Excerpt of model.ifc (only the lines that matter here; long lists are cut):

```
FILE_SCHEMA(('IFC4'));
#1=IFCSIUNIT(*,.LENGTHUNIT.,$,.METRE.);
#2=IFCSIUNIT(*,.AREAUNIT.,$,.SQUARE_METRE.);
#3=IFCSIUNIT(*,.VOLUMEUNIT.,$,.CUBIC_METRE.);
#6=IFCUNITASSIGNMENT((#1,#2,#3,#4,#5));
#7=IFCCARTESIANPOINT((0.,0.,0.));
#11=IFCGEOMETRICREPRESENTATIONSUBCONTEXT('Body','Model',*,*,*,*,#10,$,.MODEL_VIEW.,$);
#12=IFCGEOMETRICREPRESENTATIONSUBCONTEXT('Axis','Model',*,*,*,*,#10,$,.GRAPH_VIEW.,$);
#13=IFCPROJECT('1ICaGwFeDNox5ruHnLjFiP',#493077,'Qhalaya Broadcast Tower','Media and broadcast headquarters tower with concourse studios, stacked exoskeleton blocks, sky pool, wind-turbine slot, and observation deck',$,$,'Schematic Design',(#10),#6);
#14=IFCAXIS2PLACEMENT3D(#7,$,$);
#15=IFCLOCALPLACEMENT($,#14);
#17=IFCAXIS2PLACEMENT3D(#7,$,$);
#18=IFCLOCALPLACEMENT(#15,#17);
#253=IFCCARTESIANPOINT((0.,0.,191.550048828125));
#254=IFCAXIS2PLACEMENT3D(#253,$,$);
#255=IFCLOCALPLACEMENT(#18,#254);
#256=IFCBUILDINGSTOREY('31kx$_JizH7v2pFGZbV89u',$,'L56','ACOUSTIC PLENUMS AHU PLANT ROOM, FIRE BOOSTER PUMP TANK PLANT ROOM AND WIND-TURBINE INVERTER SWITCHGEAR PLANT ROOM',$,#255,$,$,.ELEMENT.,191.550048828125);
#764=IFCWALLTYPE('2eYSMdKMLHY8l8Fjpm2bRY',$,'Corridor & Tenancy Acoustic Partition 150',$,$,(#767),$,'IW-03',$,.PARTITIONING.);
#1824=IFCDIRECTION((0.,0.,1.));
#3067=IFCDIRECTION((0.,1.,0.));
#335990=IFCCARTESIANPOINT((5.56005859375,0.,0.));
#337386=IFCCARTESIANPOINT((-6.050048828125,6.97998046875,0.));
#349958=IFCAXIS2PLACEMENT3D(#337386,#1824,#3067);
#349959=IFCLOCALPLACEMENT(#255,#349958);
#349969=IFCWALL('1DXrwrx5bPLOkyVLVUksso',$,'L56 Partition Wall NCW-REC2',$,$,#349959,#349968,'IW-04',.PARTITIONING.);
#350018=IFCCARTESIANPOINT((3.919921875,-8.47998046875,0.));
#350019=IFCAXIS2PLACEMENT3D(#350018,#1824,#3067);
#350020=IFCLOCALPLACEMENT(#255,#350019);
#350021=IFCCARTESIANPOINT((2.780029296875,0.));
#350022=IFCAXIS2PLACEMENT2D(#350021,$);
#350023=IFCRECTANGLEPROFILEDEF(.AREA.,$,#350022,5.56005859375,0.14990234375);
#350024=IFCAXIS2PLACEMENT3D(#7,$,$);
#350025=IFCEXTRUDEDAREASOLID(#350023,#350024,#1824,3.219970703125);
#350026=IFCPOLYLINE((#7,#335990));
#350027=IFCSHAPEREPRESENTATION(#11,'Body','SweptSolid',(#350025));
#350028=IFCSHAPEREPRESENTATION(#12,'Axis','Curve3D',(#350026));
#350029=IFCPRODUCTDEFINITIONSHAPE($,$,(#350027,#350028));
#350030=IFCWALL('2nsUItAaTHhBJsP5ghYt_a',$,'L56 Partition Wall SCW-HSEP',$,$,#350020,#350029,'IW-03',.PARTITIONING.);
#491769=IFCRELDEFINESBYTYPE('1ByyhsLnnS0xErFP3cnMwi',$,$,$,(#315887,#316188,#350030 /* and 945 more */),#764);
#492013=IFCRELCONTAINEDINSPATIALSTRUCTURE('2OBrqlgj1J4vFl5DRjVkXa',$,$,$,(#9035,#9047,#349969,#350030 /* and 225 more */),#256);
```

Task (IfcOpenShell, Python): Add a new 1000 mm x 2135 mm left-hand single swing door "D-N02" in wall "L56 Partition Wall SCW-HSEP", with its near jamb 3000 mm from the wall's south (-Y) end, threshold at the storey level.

```python
import numpy as np
import ifcopenshell
import ifcopenshell.api.feature
import ifcopenshell.api.geometry
import ifcopenshell.api.root
import ifcopenshell.api.spatial
import ifcopenshell.geom
import ifcopenshell.util.element
import ifcopenshell.util.placement
import ifcopenshell.util.representation
import ifcopenshell.util.shape
import ifcopenshell.util.unit

model = ifcopenshell.open("model.ifc")
unit_scale = ifcopenshell.util.unit.calculate_unit_scale(model)
settings = ifcopenshell.geom.settings()


def volume(element):
    """Net volume in cubic metres, openings subtracted."""
    shape = ifcopenshell.geom.create_shape(settings, element)
    return ifcopenshell.util.shape.get_volume(shape.geometry)


wall = model.by_id(350030)
storey = ifcopenshell.util.element.get_container(wall, ifc_class="IfcBuildingStorey")
context = ifcopenshell.util.representation.get_context(model, "Model", "Body", "MODEL_VIEW")
before = volume(wall)

width, height, from_end, sill = 1, 2.135, 3, 0.0  # metres

# The wall runs along its own X axis, and the end named is its -X end.
wall_shape = ifcopenshell.geom.create_shape(settings, wall)
x, y, z = ifcopenshell.util.shape.get_vertices(wall_shape.geometry).T
start = x.min() + from_end
face, thickness = float(y.min()), float(y.max() - y.min())
wall_matrix = ifcopenshell.util.placement.get_local_placement(wall.ObjectPlacement)
level = ifcopenshell.util.placement.get_local_placement(storey.ObjectPlacement)[2, 3]


def in_wall(x, y):
    """Placement at x, y metres in the wall's axes, at sill height."""
    matrix = wall_matrix.copy()
    matrix[:, 3] = wall_matrix @ np.array([x / unit_scale, y / unit_scale, 0.0, 1.0])
    matrix[2, 3] = level + sill / unit_scale
    return matrix


# Opening: a box that overshoots both wall faces by 50 mm.
opening = ifcopenshell.api.root.create_entity(model, ifc_class="IfcOpeningElement", predefined_type="OPENING")
box = ifcopenshell.api.geometry.add_wall_representation(
    model, context=context, length=width, height=height, thickness=thickness + 0.1
)
ifcopenshell.api.geometry.assign_representation(model, product=opening, representation=box)
ifcopenshell.api.geometry.edit_object_placement(model, product=opening, matrix=in_wall(start, face - 0.05), is_si=False)
ifcopenshell.api.feature.add_feature(model, feature=opening, element=wall)

door = ifcopenshell.api.root.create_entity(model, ifc_class="IfcDoor", name="D-N02", predefined_type="DOOR")
door.OverallWidth, door.OverallHeight = width / unit_scale, height / unit_scale
door.OperationType = "SINGLE_SWING_LEFT"
body = ifcopenshell.api.geometry.add_door_representation(
    model,
    context=context,
    overall_width=door.OverallWidth,
    overall_height=door.OverallHeight,
    operation_type="SINGLE_SWING_LEFT",
    lining_properties={"LiningDepth": thickness / unit_scale, "ThresholdDepth": thickness / unit_scale},
)
ifcopenshell.api.geometry.assign_representation(model, product=door, representation=body)
ifcopenshell.api.spatial.assign_container(model, products=[door], relating_structure=storey)
ifcopenshell.api.feature.add_filling(model, opening=opening, element=door)

# The lining spans the wall, so the door starts at the wall face.
ifcopenshell.api.geometry.edit_object_placement(model, product=door, matrix=in_wall(start, face), is_si=False)

after = volume(wall)

print(f"wall volume {before:.3f} -> {after:.3f} m3")

model.write("model-out.ifc")
```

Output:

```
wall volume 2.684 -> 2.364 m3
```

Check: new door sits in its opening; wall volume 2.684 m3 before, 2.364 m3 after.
